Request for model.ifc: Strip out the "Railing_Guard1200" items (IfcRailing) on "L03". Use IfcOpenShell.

First a look at what the model holds.

```python
import ifcopenshell
import ifcopenshell.util.element

model = ifcopenshell.open("model.ifc")
print(model.schema)
storey = next(s for s in model.by_type("IfcBuildingStorey") if s.Name == "L03")
railings = [e for e in ifcopenshell.util.element.get_decomposition(storey) if e.is_a("IfcRailing")]
seen = {}
for e in railings:
    element_type = ifcopenshell.util.element.get_type(e)
    name = element_type.Name if element_type not in (None, e) else None
    seen[name] = seen.get(name, 0) + 1
for name, count in sorted(seen.items(), key=str):
    print(count, "x", name)
```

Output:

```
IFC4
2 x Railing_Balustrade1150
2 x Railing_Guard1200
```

```python
import ifcopenshell
import ifcopenshell.api.root
import ifcopenshell.util.element

model = ifcopenshell.open("model.ifc")

storey = next(s for s in model.by_type("IfcBuildingStorey") if s.Name == "L03")
railings = [e for e in ifcopenshell.util.element.get_decomposition(storey) if e.is_a("IfcRailing")]
targets = [e for e in railings if (t := ifcopenshell.util.element.get_type(e)) not in (None, e) and t.Name == "Railing_Guard1200"]

for e in targets:
    ifcopenshell.api.root.remove_product(model, product=e)
print(len(targets), "removed")

model.write("model_edited.ifc")
```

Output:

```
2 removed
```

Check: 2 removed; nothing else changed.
